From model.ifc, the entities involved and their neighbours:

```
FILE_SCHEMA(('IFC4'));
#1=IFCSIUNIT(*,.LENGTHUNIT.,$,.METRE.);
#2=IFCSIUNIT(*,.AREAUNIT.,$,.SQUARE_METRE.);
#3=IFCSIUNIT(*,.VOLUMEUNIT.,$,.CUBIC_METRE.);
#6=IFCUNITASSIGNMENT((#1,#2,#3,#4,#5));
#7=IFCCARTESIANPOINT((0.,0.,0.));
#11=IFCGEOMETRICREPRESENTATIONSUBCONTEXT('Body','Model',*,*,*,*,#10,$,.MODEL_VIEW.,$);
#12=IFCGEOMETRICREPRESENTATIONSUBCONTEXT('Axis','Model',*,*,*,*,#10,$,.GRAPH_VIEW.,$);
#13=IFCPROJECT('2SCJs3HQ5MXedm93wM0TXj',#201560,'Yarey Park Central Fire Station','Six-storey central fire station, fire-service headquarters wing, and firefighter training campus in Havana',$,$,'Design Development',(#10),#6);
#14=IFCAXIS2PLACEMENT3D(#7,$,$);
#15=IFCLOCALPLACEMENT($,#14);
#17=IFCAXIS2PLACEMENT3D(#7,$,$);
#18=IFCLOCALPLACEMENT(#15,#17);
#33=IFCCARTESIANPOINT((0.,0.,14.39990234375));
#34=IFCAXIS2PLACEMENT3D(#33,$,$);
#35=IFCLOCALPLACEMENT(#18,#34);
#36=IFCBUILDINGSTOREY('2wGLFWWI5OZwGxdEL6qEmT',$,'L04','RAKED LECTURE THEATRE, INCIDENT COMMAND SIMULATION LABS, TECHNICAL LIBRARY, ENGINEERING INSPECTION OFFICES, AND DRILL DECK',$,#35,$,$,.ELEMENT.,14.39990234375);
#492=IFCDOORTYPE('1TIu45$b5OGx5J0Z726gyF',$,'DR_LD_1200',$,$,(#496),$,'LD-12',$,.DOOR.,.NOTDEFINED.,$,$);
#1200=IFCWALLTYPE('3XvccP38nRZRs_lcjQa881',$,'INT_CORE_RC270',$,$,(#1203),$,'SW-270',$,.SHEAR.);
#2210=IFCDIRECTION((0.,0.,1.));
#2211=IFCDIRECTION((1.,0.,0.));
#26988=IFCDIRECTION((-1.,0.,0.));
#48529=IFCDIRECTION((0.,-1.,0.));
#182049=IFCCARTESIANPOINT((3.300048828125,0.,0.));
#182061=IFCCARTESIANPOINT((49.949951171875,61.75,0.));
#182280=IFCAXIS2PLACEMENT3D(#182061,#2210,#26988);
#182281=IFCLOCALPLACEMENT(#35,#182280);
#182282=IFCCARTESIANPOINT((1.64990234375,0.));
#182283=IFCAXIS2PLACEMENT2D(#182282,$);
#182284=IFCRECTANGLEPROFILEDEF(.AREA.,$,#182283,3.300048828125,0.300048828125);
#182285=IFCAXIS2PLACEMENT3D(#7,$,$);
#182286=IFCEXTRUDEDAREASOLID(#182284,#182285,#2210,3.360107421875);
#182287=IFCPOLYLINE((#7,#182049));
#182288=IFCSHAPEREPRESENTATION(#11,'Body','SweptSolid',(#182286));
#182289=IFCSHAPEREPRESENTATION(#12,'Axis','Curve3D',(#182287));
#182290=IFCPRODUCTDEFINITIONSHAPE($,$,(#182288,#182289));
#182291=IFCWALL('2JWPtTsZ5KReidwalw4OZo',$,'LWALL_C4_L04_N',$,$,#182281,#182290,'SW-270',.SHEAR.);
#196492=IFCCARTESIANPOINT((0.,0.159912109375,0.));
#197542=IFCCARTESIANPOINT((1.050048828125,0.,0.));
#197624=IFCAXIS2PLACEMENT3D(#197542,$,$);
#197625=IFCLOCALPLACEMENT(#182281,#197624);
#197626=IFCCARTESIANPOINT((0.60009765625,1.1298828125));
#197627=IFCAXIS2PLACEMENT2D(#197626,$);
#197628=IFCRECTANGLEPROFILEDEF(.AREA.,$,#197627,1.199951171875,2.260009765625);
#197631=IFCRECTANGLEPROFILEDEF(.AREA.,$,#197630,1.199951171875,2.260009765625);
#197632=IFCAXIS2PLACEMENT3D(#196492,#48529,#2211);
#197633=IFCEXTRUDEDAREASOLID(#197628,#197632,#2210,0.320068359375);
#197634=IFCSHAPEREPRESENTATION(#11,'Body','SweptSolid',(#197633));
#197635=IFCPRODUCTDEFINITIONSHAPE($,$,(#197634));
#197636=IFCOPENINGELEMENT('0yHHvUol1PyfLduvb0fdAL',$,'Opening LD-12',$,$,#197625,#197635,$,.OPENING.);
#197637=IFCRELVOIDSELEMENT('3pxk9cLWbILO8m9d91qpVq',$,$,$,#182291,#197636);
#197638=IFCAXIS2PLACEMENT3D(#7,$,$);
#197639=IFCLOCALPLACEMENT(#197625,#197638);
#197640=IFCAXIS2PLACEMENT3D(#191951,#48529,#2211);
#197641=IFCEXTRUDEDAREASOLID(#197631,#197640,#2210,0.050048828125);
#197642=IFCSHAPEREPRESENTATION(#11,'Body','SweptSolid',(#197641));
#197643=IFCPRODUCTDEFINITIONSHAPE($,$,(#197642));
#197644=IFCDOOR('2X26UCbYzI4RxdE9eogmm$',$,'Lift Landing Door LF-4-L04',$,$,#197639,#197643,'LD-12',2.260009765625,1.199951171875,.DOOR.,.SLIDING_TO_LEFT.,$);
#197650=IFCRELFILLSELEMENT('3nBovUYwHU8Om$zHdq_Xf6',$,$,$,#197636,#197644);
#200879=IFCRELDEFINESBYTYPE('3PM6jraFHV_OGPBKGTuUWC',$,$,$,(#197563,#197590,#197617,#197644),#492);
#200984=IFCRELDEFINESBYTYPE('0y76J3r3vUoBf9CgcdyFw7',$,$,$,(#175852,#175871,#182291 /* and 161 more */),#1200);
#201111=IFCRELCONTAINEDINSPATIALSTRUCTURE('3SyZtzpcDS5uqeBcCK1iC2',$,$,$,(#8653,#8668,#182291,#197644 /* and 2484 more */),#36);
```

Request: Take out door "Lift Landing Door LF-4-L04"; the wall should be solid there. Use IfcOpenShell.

```python
import ifcopenshell
import ifcopenshell.api.feature
import ifcopenshell.api.root
import ifcopenshell.geom
import ifcopenshell.util.shape

model = ifcopenshell.open("model.ifc")
settings = ifcopenshell.geom.settings()


def volume(element):
    """Net volume in cubic metres, openings subtracted."""
    shape = ifcopenshell.geom.create_shape(settings, element)
    return ifcopenshell.util.shape.get_volume(shape.geometry)


door = model.by_id(197644)
opening = door.FillsVoids[0].RelatingOpeningElement
wall = opening.VoidsElements[0].RelatingBuildingElement
before = volume(wall)

ifcopenshell.api.root.remove_product(model, product=door)
ifcopenshell.api.feature.remove_feature(model, feature=opening)

after = volume(wall)

print(f"wall volume {before:.3f} -> {after:.3f} m3")

model.write("model_v2.ifc")
```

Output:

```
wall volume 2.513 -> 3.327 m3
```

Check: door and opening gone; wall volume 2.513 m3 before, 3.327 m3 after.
